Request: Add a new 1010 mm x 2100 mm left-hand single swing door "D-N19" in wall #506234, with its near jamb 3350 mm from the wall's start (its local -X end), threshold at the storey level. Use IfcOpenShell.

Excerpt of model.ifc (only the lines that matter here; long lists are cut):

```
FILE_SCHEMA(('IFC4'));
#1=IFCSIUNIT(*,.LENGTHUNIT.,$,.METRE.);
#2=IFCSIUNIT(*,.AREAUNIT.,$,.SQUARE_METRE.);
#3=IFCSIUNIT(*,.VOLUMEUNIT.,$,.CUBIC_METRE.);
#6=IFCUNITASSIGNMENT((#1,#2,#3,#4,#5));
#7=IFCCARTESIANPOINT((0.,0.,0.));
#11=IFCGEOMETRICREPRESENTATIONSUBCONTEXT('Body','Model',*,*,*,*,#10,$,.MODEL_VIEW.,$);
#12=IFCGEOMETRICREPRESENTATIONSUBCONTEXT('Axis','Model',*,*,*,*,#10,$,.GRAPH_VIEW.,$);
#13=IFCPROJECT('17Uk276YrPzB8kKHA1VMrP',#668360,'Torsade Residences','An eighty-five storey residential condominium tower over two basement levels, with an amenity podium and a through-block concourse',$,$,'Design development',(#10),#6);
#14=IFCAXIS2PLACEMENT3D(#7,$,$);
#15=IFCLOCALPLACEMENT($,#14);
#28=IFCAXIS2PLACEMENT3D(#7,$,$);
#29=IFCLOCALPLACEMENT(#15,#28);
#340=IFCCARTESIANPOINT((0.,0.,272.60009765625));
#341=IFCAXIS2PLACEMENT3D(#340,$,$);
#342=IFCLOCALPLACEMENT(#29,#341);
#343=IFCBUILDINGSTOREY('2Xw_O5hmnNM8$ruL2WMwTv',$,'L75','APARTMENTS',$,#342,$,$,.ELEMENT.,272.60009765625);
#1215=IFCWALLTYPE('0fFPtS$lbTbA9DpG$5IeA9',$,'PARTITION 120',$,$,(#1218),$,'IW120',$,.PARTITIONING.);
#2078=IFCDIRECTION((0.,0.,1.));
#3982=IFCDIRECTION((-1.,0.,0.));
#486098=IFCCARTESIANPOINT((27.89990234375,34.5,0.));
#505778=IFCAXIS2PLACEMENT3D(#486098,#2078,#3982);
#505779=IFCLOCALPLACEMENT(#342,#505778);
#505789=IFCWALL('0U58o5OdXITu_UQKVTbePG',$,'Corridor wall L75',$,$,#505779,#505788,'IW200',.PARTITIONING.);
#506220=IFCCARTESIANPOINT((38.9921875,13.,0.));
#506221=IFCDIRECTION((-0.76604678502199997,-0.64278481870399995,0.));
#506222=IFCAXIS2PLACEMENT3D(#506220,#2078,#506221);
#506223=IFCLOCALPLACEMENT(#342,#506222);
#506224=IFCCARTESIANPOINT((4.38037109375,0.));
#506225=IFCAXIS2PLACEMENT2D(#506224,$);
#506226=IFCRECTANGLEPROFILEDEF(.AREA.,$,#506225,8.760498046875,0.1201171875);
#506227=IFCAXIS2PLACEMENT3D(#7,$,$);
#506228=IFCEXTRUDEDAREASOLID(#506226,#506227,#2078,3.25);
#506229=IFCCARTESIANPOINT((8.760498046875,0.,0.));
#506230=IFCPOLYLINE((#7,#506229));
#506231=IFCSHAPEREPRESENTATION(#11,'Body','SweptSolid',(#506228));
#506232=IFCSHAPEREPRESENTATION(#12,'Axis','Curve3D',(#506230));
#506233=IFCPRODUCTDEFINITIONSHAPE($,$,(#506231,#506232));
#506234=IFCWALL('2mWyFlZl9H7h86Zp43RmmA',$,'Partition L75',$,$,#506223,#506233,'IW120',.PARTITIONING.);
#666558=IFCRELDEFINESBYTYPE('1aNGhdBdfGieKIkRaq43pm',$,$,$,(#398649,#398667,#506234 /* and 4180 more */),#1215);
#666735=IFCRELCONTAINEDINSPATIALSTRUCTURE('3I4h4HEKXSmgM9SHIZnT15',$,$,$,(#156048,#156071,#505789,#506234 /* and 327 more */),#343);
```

```python
import numpy as np
import ifcopenshell
import ifcopenshell.api.feature
import ifcopenshell.api.geometry
import ifcopenshell.api.root
import ifcopenshell.api.spatial
import ifcopenshell.geom
import ifcopenshell.util.element
import ifcopenshell.util.placement
import ifcopenshell.util.representation
import ifcopenshell.util.shape
import ifcopenshell.util.unit

model = ifcopenshell.open("model.ifc")
unit_scale = ifcopenshell.util.unit.calculate_unit_scale(model)
settings = ifcopenshell.geom.settings()


def volume(element):
    """Net volume in cubic metres, openings subtracted."""
    shape = ifcopenshell.geom.create_shape(settings, element)
    return ifcopenshell.util.shape.get_volume(shape.geometry)


wall = model.by_guid("2mWyFlZl9H7h86Zp43RmmA")
storey = ifcopenshell.util.element.get_container(wall, ifc_class="IfcBuildingStorey")
context = ifcopenshell.util.representation.get_context(model, "Model", "Body", "MODEL_VIEW")
before = volume(wall)

width, height, from_end, sill = 1.01, 2.1, 3.35, 0.0  # metres

# The wall runs along its own X axis, and the end named is its -X end.
wall_shape = ifcopenshell.geom.create_shape(settings, wall)
x, y, z = ifcopenshell.util.shape.get_vertices(wall_shape.geometry).T
start = x.min() + from_end
face, thickness = float(y.min()), float(y.max() - y.min())
wall_matrix = ifcopenshell.util.placement.get_local_placement(wall.ObjectPlacement)
level = ifcopenshell.util.placement.get_local_placement(storey.ObjectPlacement)[2, 3]


def in_wall(x, y):
    """Placement at x, y metres in the wall's axes, at sill height."""
    matrix = wall_matrix.copy()
    matrix[:, 3] = wall_matrix @ np.array([x / unit_scale, y / unit_scale, 0.0, 1.0])
    matrix[2, 3] = level + sill / unit_scale
    return matrix


# Opening: a box that overshoots both wall faces by 50 mm.
opening = ifcopenshell.api.root.create_entity(model, ifc_class="IfcOpeningElement", predefined_type="OPENING")
box = ifcopenshell.api.geometry.add_wall_representation(
    model, context=context, length=width, height=height, thickness=thickness + 0.1
)
ifcopenshell.api.geometry.assign_representation(model, product=opening, representation=box)
ifcopenshell.api.geometry.edit_object_placement(model, product=opening, matrix=in_wall(start, face - 0.05), is_si=False)
ifcopenshell.api.feature.add_feature(model, feature=opening, element=wall)

door = ifcopenshell.api.root.create_entity(model, ifc_class="IfcDoor", name="D-N19", predefined_type="DOOR")
door.OverallWidth, door.OverallHeight = width / unit_scale, height / unit_scale
door.OperationType = "SINGLE_SWING_LEFT"
body = ifcopenshell.api.geometry.add_door_representation(
    model,
    context=context,
    overall_width=door.OverallWidth,
    overall_height=door.OverallHeight,
    operation_type="SINGLE_SWING_LEFT",
    lining_properties={"LiningDepth": thickness / unit_scale, "ThresholdDepth": thickness / unit_scale},
)
ifcopenshell.api.geometry.assign_representation(model, product=door, representation=body)
ifcopenshell.api.spatial.assign_container(model, products=[door], relating_structure=storey)
ifcopenshell.api.feature.add_filling(model, opening=opening, element=door)

# The lining spans the wall, so the door starts at the wall face.
ifcopenshell.api.geometry.edit_object_placement(model, product=door, matrix=in_wall(start, face), is_si=False)

after = volume(wall)

print(f"wall volume {before:.3f} -> {after:.3f} m3")

model.write("model-out.ifc")
```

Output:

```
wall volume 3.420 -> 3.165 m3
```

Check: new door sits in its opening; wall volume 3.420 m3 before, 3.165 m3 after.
